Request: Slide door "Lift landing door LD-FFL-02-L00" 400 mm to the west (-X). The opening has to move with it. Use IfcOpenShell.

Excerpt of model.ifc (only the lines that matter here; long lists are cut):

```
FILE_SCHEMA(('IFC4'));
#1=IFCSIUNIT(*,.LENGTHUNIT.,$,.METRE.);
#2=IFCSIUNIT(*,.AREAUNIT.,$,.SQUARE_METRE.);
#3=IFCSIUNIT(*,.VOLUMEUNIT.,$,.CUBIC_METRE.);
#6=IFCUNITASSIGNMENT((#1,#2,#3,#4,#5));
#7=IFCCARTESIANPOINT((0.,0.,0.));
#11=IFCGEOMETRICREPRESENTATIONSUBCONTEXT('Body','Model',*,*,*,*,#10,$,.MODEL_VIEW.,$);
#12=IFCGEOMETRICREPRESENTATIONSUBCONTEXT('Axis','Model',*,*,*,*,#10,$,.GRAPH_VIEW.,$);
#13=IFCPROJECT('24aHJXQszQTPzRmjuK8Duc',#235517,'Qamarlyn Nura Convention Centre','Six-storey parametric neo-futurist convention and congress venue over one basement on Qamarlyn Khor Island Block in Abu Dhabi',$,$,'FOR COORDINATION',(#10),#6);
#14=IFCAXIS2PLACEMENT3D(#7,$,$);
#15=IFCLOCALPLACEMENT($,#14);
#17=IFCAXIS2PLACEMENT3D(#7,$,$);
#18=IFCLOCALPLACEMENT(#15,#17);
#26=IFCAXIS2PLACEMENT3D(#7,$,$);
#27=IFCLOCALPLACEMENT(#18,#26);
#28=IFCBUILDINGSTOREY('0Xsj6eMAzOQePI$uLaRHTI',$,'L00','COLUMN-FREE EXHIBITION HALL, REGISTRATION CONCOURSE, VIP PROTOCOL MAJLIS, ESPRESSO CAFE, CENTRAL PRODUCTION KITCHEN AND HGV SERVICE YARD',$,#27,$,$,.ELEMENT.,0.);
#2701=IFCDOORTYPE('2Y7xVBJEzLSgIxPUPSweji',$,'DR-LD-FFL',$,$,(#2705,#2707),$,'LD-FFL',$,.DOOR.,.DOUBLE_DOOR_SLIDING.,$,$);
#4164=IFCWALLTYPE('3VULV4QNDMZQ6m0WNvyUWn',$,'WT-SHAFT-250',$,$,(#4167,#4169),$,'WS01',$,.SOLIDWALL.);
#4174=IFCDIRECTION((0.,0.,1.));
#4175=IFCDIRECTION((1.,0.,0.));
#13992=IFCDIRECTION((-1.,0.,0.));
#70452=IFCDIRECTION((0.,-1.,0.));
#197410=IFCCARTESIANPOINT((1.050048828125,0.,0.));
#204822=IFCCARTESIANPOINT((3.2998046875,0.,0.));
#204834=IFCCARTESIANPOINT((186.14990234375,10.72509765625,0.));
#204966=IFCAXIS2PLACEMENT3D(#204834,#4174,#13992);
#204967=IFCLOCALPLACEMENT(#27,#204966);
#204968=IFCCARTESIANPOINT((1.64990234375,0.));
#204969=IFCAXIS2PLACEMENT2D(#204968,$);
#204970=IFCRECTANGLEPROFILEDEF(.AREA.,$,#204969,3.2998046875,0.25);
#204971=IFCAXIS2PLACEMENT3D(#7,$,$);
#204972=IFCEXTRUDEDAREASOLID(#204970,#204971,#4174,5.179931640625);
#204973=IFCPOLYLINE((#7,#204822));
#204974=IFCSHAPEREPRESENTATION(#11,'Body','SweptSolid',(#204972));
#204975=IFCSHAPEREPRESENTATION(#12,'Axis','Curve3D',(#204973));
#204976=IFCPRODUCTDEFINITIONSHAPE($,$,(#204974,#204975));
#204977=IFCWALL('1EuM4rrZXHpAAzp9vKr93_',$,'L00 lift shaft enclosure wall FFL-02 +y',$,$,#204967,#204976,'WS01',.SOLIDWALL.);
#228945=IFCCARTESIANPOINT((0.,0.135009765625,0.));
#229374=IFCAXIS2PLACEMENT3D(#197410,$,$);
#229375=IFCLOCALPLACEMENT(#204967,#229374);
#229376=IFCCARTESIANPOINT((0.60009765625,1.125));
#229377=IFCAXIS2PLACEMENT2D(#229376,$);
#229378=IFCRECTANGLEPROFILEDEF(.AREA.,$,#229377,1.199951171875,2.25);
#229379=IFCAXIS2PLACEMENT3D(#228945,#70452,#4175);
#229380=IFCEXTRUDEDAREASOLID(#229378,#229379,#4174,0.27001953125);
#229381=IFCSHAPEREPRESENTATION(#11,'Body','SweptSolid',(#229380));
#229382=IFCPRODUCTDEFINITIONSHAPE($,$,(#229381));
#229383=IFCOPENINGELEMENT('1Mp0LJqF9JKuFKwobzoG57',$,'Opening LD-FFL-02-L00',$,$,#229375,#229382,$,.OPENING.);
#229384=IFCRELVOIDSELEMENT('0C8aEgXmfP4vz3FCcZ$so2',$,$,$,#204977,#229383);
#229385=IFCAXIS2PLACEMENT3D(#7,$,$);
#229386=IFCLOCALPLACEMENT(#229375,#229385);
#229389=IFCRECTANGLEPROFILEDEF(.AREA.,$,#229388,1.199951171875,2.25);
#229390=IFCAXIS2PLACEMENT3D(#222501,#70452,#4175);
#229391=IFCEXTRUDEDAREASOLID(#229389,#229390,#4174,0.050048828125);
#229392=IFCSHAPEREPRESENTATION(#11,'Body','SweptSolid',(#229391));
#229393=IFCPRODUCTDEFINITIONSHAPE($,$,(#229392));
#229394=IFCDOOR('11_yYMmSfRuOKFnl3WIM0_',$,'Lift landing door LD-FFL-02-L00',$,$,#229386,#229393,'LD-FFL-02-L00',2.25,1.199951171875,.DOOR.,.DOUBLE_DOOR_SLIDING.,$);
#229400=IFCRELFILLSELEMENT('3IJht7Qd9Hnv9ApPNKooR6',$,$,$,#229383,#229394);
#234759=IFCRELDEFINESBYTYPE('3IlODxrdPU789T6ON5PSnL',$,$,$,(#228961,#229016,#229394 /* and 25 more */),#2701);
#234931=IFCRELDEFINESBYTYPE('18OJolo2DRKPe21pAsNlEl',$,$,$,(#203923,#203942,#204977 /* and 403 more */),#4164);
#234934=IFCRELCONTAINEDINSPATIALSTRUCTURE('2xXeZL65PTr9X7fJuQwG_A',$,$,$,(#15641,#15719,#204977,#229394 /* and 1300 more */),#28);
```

```python
import ifcopenshell
import ifcopenshell.api.geometry
import ifcopenshell.util.placement
import ifcopenshell.util.unit

model = ifcopenshell.open("model.ifc")
unit_scale = ifcopenshell.util.unit.calculate_unit_scale(model)

door = model.by_guid("11_yYMmSfRuOKFnl3WIM0_")
opening = door.FillsVoids[0].RelatingOpeningElement
wall = opening.VoidsElements[0].RelatingBuildingElement

wall_matrix = ifcopenshell.util.placement.get_local_placement(wall.ObjectPlacement)
shift = wall_matrix[:3, 0] * 0.4 / unit_scale
before = ifcopenshell.util.placement.get_local_placement(door.ObjectPlacement)[:3, 3].copy()

# The door is placed relative to its opening, so it follows when the opening moves.
matrix = ifcopenshell.util.placement.get_local_placement(opening.ObjectPlacement)
matrix[:3, 3] += shift
ifcopenshell.api.geometry.edit_object_placement(
    model, product=opening, matrix=matrix, is_si=False, should_transform_children=True
)

after = ifcopenshell.util.placement.get_local_placement(door.ObjectPlacement)[:3, 3]
print("door moved by", (after - before).round(3) + 0.0)

model.write("model_rev.ifc")
```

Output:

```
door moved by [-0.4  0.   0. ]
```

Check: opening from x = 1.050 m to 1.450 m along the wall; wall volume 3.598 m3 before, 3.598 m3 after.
